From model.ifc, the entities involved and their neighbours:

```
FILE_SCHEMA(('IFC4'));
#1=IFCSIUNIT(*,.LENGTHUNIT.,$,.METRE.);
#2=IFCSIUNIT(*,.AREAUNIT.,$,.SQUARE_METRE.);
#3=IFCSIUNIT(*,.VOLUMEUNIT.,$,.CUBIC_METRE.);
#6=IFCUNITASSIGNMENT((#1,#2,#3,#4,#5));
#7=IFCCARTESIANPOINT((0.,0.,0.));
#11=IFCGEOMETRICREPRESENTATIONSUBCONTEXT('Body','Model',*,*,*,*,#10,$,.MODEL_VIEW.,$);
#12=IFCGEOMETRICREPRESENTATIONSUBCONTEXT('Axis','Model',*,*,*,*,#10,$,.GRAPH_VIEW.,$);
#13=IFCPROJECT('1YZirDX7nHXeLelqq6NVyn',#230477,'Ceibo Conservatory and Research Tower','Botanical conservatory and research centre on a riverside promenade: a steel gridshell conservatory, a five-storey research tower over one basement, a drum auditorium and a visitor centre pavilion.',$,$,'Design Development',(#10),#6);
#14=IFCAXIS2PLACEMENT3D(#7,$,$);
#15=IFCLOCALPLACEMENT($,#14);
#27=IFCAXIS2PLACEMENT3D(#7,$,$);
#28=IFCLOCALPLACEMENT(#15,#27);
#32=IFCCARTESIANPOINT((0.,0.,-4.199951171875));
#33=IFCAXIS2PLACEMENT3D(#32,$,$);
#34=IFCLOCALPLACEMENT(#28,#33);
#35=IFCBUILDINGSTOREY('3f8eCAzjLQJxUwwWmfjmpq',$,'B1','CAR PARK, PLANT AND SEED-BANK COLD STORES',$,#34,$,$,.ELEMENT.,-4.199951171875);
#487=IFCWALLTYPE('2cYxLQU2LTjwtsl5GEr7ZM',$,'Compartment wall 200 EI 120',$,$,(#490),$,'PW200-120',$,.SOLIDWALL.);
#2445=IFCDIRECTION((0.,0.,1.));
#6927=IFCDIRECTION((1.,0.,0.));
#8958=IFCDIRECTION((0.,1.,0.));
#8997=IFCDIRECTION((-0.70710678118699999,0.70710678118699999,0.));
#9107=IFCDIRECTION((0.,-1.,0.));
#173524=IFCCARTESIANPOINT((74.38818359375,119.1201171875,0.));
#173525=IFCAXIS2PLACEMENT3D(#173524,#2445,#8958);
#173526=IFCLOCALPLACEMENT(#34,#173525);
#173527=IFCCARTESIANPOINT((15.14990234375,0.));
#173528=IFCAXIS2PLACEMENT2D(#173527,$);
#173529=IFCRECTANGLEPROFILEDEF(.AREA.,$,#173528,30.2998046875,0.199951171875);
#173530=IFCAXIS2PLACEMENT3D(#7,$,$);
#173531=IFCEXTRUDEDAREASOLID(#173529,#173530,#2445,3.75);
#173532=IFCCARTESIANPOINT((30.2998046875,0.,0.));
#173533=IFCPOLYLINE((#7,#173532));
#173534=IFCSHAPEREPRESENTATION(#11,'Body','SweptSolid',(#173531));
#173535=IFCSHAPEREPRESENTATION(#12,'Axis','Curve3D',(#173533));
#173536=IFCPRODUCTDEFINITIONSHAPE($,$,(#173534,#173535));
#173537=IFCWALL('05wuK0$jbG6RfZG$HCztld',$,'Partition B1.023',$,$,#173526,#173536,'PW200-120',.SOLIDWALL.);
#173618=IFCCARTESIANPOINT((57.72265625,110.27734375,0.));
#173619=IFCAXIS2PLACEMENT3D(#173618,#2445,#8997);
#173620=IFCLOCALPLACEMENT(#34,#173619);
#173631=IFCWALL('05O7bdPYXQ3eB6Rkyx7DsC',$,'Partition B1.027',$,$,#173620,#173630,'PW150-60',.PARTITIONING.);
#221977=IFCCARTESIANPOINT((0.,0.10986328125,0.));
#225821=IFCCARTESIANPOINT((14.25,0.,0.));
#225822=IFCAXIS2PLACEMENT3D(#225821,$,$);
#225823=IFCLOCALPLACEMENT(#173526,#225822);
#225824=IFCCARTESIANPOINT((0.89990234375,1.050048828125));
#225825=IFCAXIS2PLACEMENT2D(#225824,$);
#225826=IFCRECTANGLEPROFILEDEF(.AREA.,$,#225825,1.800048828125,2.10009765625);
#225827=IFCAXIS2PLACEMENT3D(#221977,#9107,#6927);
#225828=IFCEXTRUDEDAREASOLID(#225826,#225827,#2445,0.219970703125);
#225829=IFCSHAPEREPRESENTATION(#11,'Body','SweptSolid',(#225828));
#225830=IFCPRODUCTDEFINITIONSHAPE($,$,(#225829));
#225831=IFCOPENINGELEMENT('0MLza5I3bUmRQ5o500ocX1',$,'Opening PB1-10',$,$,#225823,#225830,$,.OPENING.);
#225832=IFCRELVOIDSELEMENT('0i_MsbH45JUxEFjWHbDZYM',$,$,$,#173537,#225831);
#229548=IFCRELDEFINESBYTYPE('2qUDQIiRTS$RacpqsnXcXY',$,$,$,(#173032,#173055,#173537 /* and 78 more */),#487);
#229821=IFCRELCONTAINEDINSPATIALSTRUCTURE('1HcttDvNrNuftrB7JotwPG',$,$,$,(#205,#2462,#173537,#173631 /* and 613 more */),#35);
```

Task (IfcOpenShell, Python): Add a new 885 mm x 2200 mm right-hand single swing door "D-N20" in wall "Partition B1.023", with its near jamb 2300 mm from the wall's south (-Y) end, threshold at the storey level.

```python
import numpy as np
import ifcopenshell
import ifcopenshell.api.feature
import ifcopenshell.api.geometry
import ifcopenshell.api.root
import ifcopenshell.api.spatial
import ifcopenshell.geom
import ifcopenshell.util.element
import ifcopenshell.util.placement
import ifcopenshell.util.representation
import ifcopenshell.util.shape
import ifcopenshell.util.unit

model = ifcopenshell.open("model.ifc")
unit_scale = ifcopenshell.util.unit.calculate_unit_scale(model)
settings = ifcopenshell.geom.settings()


def volume(element):
    """Net volume in cubic metres, openings subtracted."""
    shape = ifcopenshell.geom.create_shape(settings, element)
    return ifcopenshell.util.shape.get_volume(shape.geometry)


wall = model.by_guid("05wuK0$jbG6RfZG$HCztld")
storey = ifcopenshell.util.element.get_container(wall, ifc_class="IfcBuildingStorey")
context = ifcopenshell.util.representation.get_context(model, "Model", "Body", "MODEL_VIEW")
before = volume(wall)

width, height, from_end, sill = 0.885, 2.2, 2.3, 0.0  # metres

# The wall runs along its own X axis, and the end named is its -X end.
wall_shape = ifcopenshell.geom.create_shape(settings, wall)
x, y, z = ifcopenshell.util.shape.get_vertices(wall_shape.geometry).T
start = x.min() + from_end
face, thickness = float(y.min()), float(y.max() - y.min())
wall_matrix = ifcopenshell.util.placement.get_local_placement(wall.ObjectPlacement)
level = ifcopenshell.util.placement.get_local_placement(storey.ObjectPlacement)[2, 3]


def in_wall(x, y):
    """Placement at x, y metres in the wall's axes, at sill height."""
    matrix = wall_matrix.copy()
    matrix[:, 3] = wall_matrix @ np.array([x / unit_scale, y / unit_scale, 0.0, 1.0])
    matrix[2, 3] = level + sill / unit_scale
    return matrix


# Opening: a box that overshoots both wall faces by 50 mm.
opening = ifcopenshell.api.root.create_entity(model, ifc_class="IfcOpeningElement", predefined_type="OPENING")
box = ifcopenshell.api.geometry.add_wall_representation(
    model, context=context, length=width, height=height, thickness=thickness + 0.1
)
ifcopenshell.api.geometry.assign_representation(model, product=opening, representation=box)
ifcopenshell.api.geometry.edit_object_placement(model, product=opening, matrix=in_wall(start, face - 0.05), is_si=False)
ifcopenshell.api.feature.add_feature(model, feature=opening, element=wall)

door = ifcopenshell.api.root.create_entity(model, ifc_class="IfcDoor", name="D-N20", predefined_type="DOOR")
door.OverallWidth, door.OverallHeight = width / unit_scale, height / unit_scale
door.OperationType = "SINGLE_SWING_RIGHT"
body = ifcopenshell.api.geometry.add_door_representation(
    model,
    context=context,
    overall_width=door.OverallWidth,
    overall_height=door.OverallHeight,
    operation_type="SINGLE_SWING_RIGHT",
    lining_properties={"LiningDepth": thickness / unit_scale, "ThresholdDepth": thickness / unit_scale},
)
ifcopenshell.api.geometry.assign_representation(model, product=door, representation=body)
ifcopenshell.api.spatial.assign_container(model, products=[door], relating_structure=storey)
ifcopenshell.api.feature.add_filling(model, opening=opening, element=door)

# The lining spans the wall, so the door starts at the wall face.
ifcopenshell.api.geometry.edit_object_placement(model, product=door, matrix=in_wall(start, face), is_si=False)

after = volume(wall)

print(f"wall volume {before:.3f} -> {after:.3f} m3")

model.write("model_v2.ifc")
```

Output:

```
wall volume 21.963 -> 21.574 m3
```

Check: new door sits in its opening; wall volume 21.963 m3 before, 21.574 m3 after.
